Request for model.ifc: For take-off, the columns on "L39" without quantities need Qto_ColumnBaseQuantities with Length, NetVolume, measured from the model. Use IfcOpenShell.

First a look at what the model holds.

```python
import ifcopenshell
import ifcopenshell.util.element
import ifcopenshell.util.unit

model = ifcopenshell.open("model.ifc")
print(model.schema)
for unit_type in ("LENGTHUNIT", "AREAUNIT", "VOLUMEUNIT"):
    print(unit_type, ifcopenshell.util.unit.calculate_unit_scale(model, unit_type))
storey = next(s for s in model.by_type("IfcBuildingStorey") if s.Name == "L39")
columns = [e for e in ifcopenshell.util.element.get_decomposition(storey) if e.is_a("IfcColumn")]
for e in sorted(columns, key=lambda e: e.id()):
    print(e.id(), e.is_a(), e.Name, list(ifcopenshell.util.element.get_psets(e, qtos_only=True)), sep=" | ")
```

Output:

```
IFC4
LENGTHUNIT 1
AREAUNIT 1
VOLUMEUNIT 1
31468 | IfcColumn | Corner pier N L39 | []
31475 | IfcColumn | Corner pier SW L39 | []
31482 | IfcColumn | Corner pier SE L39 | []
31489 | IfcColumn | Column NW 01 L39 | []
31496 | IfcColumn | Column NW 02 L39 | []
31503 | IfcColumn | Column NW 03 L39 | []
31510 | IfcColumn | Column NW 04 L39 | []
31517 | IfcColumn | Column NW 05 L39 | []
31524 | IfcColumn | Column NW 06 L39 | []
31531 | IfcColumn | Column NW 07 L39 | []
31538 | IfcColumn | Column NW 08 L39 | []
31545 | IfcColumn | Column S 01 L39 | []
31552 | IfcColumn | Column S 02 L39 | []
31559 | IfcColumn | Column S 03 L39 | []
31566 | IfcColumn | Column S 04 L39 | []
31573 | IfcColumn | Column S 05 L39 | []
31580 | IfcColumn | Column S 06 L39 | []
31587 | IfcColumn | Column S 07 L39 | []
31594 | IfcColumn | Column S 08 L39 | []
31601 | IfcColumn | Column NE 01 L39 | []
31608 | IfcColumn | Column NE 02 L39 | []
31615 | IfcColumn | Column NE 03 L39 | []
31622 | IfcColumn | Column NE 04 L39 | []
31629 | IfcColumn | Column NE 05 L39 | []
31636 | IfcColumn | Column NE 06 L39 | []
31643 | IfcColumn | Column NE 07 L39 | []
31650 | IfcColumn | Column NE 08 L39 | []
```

```python
import ifcopenshell
import ifcopenshell.api.pset
import ifcopenshell.geom
import ifcopenshell.util.element
import ifcopenshell.util.shape
import ifcopenshell.util.unit

model = ifcopenshell.open("model.ifc")
unit_scale = ifcopenshell.util.unit.calculate_unit_scale(model)
volume_scale = ifcopenshell.util.unit.calculate_unit_scale(model, "VOLUMEUNIT")
settings = ifcopenshell.geom.settings()

storey = next(s for s in model.by_type("IfcBuildingStorey") if s.Name == "L39")
columns = [e for e in ifcopenshell.util.element.get_decomposition(storey) if e.is_a("IfcColumn")]

for e in sorted(columns, key=lambda e: e.id()):
    if ifcopenshell.util.element.get_psets(e, qtos_only=True, should_inherit=False):
        continue
    # Geometry comes back in metres, in the element's own axes.
    shape = ifcopenshell.geom.create_shape(settings, e)
    values = {
        "Length": ifcopenshell.util.shape.get_z(shape.geometry) / unit_scale,
        "NetVolume": ifcopenshell.util.shape.get_volume(shape.geometry) / volume_scale,
    }
    qto = ifcopenshell.api.pset.add_qto(model, product=e, name="Qto_ColumnBaseQuantities")
    ifcopenshell.api.pset.edit_qto(model, qto=qto, properties=values)
    print(e.id(), {k: round(v, 3) for k, v in values.items()})

model.write("model_updated.ifc")
```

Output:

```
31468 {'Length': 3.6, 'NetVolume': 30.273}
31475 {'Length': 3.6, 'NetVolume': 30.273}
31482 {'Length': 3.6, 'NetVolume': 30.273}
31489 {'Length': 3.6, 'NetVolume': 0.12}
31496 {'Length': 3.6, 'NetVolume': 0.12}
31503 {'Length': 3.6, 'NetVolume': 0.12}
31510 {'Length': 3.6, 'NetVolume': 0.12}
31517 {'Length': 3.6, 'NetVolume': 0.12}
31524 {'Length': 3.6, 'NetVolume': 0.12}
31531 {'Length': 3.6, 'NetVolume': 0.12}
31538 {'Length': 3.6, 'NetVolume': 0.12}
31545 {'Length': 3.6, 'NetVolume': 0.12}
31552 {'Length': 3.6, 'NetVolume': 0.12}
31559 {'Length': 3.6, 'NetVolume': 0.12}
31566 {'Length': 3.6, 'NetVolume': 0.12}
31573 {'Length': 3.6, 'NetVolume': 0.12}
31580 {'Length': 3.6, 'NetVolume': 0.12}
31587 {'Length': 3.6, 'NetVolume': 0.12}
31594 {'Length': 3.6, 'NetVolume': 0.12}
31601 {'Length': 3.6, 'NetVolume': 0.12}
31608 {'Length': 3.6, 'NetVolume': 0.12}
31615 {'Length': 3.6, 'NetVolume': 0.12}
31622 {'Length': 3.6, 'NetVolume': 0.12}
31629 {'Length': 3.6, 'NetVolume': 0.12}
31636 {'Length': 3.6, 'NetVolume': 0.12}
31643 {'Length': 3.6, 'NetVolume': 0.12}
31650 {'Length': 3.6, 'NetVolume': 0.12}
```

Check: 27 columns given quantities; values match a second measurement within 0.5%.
